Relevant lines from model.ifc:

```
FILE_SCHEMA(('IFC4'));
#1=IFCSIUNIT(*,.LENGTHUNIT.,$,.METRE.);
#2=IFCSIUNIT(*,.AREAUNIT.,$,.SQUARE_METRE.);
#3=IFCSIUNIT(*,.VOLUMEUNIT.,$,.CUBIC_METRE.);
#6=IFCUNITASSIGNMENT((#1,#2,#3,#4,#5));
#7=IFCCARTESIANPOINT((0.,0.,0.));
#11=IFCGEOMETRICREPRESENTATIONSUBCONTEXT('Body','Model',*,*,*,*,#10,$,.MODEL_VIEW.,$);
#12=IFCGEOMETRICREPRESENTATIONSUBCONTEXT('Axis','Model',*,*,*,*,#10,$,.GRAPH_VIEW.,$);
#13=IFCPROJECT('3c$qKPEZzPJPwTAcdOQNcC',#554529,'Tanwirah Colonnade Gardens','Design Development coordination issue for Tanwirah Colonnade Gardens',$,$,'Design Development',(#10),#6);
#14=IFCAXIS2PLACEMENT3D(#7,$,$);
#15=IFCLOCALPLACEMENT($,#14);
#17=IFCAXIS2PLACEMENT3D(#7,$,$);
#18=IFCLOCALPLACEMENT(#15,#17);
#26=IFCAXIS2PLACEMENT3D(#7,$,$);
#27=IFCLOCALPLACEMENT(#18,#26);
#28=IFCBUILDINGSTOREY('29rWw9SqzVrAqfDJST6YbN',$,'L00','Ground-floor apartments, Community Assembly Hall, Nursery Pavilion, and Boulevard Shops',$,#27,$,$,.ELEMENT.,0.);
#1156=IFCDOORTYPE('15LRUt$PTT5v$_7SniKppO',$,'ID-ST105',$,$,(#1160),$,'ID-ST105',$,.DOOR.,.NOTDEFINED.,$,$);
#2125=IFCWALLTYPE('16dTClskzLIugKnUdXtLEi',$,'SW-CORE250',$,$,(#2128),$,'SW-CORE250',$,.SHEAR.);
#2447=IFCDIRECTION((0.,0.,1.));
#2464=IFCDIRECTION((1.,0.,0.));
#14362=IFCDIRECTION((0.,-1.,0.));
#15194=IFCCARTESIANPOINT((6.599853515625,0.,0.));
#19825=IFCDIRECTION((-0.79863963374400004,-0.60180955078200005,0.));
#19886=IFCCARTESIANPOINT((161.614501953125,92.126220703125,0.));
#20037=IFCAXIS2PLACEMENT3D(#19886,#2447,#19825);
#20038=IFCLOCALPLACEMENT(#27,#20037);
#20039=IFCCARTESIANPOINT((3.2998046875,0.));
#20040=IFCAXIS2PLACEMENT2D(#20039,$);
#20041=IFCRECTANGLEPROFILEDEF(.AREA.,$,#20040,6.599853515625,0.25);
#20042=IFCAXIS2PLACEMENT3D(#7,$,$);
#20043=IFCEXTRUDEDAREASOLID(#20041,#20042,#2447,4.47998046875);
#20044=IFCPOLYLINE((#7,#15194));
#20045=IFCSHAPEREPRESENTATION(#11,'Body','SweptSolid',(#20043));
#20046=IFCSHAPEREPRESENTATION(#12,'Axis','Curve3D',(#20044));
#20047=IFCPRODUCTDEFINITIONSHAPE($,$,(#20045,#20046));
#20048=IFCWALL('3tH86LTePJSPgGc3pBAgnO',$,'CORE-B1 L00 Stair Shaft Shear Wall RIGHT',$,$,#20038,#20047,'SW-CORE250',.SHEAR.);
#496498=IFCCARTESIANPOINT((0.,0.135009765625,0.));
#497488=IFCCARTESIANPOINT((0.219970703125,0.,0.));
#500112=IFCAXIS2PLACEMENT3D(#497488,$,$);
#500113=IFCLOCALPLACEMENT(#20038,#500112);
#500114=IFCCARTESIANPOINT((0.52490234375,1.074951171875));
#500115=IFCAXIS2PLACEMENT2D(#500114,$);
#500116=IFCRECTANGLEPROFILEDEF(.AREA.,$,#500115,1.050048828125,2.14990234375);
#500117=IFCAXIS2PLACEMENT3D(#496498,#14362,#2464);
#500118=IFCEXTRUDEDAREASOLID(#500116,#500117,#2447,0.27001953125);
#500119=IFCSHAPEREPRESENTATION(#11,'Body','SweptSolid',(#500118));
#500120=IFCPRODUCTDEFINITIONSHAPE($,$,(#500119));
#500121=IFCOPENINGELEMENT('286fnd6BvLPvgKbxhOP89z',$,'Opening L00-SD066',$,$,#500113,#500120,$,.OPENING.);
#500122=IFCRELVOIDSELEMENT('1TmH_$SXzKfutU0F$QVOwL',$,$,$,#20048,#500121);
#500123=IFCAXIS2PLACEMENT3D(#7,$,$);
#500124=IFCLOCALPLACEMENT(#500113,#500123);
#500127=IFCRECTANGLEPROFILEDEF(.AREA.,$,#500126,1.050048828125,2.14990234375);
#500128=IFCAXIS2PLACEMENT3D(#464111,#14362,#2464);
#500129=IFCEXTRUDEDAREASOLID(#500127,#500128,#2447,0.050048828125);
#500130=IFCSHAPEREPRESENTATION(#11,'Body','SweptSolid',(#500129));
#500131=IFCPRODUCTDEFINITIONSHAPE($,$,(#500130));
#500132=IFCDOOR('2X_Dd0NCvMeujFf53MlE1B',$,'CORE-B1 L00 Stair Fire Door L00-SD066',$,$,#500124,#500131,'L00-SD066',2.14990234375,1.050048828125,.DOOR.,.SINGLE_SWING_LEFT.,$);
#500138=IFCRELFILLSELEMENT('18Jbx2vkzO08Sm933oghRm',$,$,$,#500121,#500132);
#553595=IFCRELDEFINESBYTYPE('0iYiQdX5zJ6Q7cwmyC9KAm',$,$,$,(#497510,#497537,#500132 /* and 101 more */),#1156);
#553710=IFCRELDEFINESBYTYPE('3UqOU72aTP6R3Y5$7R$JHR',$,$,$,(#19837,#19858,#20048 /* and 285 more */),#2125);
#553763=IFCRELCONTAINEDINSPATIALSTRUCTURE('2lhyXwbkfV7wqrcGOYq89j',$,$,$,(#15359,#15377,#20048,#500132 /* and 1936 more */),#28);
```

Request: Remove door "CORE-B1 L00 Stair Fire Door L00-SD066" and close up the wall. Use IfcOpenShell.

```python
import ifcopenshell
import ifcopenshell.api.feature
import ifcopenshell.api.root
import ifcopenshell.geom
import ifcopenshell.util.shape

model = ifcopenshell.open("model.ifc")
settings = ifcopenshell.geom.settings()


def volume(element):
    """Net volume in cubic metres, openings subtracted."""
    shape = ifcopenshell.geom.create_shape(settings, element)
    return ifcopenshell.util.shape.get_volume(shape.geometry)


door = model.by_id(500132)
opening = door.FillsVoids[0].RelatingOpeningElement
wall = opening.VoidsElements[0].RelatingBuildingElement
before = volume(wall)

ifcopenshell.api.root.remove_product(model, product=door)
ifcopenshell.api.feature.remove_feature(model, feature=opening)

after = volume(wall)

print(f"wall volume {before:.3f} -> {after:.3f} m3")

model.write("model_rev.ifc")
```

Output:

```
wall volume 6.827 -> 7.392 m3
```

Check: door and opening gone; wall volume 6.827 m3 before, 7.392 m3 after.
